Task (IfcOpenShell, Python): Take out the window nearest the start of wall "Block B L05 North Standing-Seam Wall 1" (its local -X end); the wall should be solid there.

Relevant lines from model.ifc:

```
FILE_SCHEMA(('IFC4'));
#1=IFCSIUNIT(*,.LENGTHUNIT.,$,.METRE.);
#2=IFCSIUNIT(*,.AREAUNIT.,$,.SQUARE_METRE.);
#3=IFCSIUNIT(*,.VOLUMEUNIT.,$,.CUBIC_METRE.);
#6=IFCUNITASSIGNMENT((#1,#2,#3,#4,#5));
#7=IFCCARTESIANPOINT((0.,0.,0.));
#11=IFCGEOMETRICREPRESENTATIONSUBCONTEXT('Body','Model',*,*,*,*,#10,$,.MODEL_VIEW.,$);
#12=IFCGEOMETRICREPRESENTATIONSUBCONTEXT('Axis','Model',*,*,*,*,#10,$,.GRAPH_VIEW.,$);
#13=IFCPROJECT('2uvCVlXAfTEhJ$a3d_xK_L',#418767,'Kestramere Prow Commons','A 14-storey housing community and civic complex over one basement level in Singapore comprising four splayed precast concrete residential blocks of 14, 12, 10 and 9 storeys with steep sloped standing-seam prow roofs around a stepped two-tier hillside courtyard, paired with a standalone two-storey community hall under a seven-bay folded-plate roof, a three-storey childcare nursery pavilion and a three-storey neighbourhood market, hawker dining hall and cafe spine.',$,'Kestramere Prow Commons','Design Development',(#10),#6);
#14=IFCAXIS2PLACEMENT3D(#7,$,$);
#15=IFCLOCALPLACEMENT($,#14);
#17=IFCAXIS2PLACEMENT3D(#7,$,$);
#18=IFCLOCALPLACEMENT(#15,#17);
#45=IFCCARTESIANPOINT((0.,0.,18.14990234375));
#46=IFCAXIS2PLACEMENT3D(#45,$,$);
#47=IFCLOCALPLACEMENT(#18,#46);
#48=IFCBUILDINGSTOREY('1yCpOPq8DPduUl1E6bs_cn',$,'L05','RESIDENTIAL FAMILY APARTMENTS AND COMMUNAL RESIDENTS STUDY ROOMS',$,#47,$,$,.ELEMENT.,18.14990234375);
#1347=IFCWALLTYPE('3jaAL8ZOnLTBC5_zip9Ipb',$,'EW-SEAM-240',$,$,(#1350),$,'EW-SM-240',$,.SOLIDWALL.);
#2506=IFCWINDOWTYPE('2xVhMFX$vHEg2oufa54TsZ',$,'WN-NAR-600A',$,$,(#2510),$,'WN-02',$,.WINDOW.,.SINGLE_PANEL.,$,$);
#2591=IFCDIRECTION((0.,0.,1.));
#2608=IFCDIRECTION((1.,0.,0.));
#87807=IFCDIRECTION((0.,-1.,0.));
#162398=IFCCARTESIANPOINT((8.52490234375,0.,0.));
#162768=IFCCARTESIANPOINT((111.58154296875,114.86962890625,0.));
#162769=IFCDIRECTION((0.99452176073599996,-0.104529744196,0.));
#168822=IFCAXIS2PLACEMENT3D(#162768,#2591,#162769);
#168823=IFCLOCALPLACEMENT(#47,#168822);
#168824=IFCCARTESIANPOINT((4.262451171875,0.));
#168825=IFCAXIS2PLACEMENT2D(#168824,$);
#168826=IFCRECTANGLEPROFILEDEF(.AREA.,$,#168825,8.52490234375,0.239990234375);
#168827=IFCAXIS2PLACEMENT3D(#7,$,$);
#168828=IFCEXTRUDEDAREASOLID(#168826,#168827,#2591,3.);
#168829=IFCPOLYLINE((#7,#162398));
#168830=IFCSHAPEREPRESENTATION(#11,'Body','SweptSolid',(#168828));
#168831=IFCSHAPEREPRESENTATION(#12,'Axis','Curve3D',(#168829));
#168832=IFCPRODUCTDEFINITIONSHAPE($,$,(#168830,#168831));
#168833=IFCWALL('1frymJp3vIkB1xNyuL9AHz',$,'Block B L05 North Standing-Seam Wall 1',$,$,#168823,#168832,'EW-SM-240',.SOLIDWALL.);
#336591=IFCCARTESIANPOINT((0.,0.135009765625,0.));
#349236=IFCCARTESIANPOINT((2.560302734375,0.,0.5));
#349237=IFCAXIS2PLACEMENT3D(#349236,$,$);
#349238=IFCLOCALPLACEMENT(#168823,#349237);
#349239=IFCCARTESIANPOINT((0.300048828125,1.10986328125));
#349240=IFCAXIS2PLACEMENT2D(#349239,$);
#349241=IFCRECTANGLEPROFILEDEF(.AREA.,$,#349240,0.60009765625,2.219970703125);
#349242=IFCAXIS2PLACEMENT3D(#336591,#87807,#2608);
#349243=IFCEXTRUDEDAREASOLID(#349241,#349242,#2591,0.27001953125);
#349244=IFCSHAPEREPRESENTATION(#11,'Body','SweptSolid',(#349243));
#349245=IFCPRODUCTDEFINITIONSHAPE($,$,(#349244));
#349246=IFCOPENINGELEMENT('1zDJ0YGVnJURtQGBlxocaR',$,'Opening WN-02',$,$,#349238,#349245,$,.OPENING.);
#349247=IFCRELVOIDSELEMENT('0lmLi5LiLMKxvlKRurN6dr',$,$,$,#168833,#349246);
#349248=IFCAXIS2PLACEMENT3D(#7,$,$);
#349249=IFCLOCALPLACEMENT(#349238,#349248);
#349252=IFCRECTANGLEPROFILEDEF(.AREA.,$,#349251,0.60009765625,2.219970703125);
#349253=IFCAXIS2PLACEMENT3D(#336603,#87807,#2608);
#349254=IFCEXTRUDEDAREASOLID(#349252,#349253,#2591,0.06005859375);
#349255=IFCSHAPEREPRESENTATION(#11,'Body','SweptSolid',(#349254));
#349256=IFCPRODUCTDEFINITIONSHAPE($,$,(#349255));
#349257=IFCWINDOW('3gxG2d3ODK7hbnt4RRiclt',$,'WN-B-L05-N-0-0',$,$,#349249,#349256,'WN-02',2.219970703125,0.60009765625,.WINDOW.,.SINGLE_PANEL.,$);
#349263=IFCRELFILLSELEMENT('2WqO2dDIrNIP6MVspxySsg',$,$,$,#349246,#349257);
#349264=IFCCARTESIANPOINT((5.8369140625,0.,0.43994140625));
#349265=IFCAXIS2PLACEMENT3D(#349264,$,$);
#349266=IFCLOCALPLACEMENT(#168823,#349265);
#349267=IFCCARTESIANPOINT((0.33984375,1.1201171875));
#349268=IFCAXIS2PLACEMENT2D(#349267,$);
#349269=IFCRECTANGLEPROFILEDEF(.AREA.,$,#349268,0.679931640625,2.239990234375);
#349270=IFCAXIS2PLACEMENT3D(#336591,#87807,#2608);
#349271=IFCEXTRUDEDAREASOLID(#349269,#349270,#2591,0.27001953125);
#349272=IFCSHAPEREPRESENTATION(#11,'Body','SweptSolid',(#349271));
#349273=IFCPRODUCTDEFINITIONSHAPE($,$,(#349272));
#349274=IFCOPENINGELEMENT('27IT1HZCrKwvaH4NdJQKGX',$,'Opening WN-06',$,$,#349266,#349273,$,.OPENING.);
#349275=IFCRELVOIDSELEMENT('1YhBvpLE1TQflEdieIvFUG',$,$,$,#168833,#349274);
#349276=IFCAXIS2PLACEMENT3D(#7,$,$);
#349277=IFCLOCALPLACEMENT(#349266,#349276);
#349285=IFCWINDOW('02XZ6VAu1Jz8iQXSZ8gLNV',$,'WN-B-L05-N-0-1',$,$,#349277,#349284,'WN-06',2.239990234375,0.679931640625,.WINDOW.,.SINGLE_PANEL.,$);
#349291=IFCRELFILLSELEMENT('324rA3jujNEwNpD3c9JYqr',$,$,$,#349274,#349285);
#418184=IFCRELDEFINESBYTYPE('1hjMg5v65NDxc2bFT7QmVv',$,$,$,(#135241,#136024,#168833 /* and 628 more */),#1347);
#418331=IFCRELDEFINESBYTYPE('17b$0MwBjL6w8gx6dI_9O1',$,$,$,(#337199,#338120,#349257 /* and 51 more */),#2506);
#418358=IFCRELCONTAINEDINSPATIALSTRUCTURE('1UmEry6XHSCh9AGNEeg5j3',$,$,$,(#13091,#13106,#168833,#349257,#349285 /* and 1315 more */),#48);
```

```python
import ifcopenshell
import ifcopenshell.api.feature
import ifcopenshell.api.root
import ifcopenshell.geom
import ifcopenshell.util.shape

model = ifcopenshell.open("model.ifc")
settings = ifcopenshell.geom.settings()


def volume(element):
    """Net volume in cubic metres, openings subtracted."""
    shape = ifcopenshell.geom.create_shape(settings, element)
    return ifcopenshell.util.shape.get_volume(shape.geometry)


window = model.by_guid("3gxG2d3ODK7hbnt4RRiclt")
opening = window.FillsVoids[0].RelatingOpeningElement
wall = opening.VoidsElements[0].RelatingBuildingElement
before = volume(wall)

ifcopenshell.api.root.remove_product(model, product=window)
ifcopenshell.api.feature.remove_feature(model, feature=opening)

after = volume(wall)

print(f"wall volume {before:.3f} -> {after:.3f} m3")

model.write("model_v2.ifc")
```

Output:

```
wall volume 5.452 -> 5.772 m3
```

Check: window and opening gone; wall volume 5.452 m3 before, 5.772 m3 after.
